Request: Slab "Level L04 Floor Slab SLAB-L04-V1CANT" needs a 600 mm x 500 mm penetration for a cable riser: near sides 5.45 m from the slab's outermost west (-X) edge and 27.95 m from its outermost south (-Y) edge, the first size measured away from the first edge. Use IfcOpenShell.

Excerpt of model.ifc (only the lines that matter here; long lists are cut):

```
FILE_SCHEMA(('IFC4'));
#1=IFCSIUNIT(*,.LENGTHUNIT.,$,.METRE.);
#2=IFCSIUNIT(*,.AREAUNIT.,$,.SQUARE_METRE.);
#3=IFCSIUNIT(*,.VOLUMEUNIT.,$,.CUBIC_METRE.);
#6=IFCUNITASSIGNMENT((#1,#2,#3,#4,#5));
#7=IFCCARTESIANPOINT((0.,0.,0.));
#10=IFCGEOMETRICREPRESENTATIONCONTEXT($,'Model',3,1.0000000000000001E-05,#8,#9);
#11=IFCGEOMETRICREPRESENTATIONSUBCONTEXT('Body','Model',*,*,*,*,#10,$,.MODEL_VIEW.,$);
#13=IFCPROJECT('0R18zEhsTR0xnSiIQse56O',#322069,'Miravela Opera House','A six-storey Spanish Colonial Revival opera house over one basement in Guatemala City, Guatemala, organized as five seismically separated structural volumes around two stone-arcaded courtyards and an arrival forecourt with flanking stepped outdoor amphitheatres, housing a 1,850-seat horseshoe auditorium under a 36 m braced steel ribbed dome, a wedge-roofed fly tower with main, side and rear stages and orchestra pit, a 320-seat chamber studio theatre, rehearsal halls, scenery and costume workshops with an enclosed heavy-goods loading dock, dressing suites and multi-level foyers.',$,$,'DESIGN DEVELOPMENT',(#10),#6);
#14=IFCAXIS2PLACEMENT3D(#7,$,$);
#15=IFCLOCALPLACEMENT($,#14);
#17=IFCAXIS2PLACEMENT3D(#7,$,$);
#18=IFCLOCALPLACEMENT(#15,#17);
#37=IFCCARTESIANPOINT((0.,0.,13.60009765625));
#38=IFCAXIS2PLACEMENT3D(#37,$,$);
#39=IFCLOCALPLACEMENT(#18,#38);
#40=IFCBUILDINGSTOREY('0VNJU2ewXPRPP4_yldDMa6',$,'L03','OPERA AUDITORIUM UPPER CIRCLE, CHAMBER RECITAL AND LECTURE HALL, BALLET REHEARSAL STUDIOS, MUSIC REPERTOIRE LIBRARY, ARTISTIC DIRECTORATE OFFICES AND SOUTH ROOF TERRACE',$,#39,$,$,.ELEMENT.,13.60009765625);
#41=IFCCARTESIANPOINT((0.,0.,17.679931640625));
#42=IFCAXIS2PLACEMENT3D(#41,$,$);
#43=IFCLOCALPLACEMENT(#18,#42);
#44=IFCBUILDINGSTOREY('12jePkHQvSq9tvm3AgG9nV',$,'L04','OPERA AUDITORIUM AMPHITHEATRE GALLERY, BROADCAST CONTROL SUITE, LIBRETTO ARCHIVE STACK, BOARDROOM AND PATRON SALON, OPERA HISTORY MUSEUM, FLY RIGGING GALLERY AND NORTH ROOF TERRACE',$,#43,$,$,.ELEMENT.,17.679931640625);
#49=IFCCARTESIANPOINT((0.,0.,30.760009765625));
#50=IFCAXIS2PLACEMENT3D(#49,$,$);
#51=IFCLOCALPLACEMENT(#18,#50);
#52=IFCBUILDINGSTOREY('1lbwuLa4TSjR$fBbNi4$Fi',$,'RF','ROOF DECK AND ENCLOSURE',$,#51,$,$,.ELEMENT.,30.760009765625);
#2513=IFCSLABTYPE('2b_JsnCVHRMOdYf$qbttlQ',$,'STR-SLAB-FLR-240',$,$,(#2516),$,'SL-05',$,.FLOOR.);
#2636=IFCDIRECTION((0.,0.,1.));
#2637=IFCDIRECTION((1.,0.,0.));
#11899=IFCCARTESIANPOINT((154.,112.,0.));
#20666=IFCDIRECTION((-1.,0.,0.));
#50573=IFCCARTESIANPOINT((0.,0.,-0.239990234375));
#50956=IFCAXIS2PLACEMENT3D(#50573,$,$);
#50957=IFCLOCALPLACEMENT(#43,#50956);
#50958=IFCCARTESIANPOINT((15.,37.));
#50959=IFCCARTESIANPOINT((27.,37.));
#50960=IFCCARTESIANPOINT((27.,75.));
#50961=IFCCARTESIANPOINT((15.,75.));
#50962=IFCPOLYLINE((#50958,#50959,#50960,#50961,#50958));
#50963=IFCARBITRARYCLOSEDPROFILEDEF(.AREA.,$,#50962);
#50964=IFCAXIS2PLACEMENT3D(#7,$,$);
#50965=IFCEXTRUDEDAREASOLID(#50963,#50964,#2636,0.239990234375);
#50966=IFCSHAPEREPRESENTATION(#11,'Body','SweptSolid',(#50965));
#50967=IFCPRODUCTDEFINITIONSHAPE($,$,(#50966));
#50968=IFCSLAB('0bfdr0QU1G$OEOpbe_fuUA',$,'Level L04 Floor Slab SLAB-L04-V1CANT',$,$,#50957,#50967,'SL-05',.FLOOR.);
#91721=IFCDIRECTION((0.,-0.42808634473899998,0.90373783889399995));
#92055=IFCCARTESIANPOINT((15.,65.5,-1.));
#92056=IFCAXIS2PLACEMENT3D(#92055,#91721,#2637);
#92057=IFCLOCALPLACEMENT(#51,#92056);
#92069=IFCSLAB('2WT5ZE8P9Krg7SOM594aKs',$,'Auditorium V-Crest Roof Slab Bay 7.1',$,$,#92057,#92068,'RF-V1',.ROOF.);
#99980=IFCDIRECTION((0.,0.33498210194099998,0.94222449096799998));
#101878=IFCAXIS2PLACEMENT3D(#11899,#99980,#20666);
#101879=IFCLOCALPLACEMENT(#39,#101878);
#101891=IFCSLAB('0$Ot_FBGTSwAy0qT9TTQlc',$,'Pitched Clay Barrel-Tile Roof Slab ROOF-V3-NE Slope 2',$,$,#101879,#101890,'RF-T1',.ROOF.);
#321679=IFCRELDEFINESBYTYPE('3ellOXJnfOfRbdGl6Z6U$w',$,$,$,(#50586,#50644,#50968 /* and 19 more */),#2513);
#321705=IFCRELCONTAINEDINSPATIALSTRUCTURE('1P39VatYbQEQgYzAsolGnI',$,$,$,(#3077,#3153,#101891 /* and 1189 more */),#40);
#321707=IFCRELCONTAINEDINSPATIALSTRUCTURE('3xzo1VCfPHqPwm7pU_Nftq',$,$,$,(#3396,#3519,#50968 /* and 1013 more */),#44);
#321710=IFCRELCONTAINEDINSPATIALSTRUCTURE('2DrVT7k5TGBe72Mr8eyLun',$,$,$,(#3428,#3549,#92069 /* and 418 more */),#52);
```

```python
import numpy as np
import ifcopenshell
import ifcopenshell.api.feature
import ifcopenshell.api.geometry
import ifcopenshell.api.root
import ifcopenshell.geom
import ifcopenshell.util.placement
import ifcopenshell.util.representation
import ifcopenshell.util.shape
import ifcopenshell.util.unit

model = ifcopenshell.open("model.ifc")
unit_scale = ifcopenshell.util.unit.calculate_unit_scale(model)
settings = ifcopenshell.geom.settings()


def volume(element):
    """Net volume in cubic metres, openings subtracted."""
    shape = ifcopenshell.geom.create_shape(settings, element)
    return ifcopenshell.util.shape.get_volume(shape.geometry)


slab = model.by_guid("0bfdr0QU1G$OEOpbe_fuUA")
before = volume(slab)

# Extent in the slab's own axes, in metres. The edges named are its -X and -Y sides.
slab_shape = ifcopenshell.geom.create_shape(settings, slab)
vertices = ifcopenshell.util.shape.get_vertices(slab_shape.geometry)
x_min, y_min, bottom = vertices.min(axis=0)
top = vertices[:, 2].max()

opening = ifcopenshell.api.root.create_entity(model, ifc_class="IfcOpeningElement", name="Cable riser opening", predefined_type="OPENING")
context = ifcopenshell.util.representation.get_context(model, "Model", "Body", "MODEL_VIEW")
width, depth = 0.6, 0.5
outline = [(0.0, 0.0), (width, 0.0), (width, depth), (0.0, depth), (0.0, 0.0)]
# Overshoot both faces by 50 mm so the cut is clean.
shape = ifcopenshell.api.geometry.add_slab_representation(
    model, context=context, depth=top - bottom + 0.1, polyline=outline
)
ifcopenshell.api.geometry.assign_representation(model, product=opening, representation=shape)

matrix = ifcopenshell.util.placement.get_local_placement(slab.ObjectPlacement)
matrix[:, 3] = matrix @ np.append(np.array([x_min + 5.45, y_min + 27.95, bottom - 0.05]) / unit_scale, 1.0)
ifcopenshell.api.geometry.edit_object_placement(model, product=opening, matrix=matrix, is_si=False)
ifcopenshell.api.feature.add_feature(model, feature=opening, element=slab)

after = volume(slab)

print(f"slab volume {before:.3f} -> {after:.3f} m3")

model.write("model_edited.ifc")
```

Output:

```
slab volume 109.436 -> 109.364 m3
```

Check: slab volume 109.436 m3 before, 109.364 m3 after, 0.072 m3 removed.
